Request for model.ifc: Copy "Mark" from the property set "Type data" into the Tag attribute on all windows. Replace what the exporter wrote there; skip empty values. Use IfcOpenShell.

First a look at what the model holds.

```python
import ifcopenshell
import ifcopenshell.util.element

model = ifcopenshell.open("model.ifc")
print(model.schema)
windows = model.by_type("IfcWindow")
print(len(windows), "windows")
for e in windows[:8]:
    source = ifcopenshell.util.element.get_pset(e, "Type data", "Mark")
    target = e.Tag
    print(e.id(), repr(source), repr(target), sep=" | ")
```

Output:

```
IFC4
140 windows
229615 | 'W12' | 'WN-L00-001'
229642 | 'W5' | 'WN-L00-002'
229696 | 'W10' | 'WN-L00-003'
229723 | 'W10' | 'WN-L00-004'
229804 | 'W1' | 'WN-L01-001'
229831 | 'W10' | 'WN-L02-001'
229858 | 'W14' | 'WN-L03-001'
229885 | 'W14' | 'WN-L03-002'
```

```python
import ifcopenshell
import ifcopenshell.util.element

model = ifcopenshell.open("model.ifc")

count = 0
for e in model.by_type("IfcWindow"):
    value = ifcopenshell.util.element.get_pset(e, "Type data", "Mark")
    current = e.Tag
    if not value or not value.strip() or current == value:
        continue
    e.Tag = value
    count += 1

print(count, "windows updated")

model.write("model-out.ifc")
```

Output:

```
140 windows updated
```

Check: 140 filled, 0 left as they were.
